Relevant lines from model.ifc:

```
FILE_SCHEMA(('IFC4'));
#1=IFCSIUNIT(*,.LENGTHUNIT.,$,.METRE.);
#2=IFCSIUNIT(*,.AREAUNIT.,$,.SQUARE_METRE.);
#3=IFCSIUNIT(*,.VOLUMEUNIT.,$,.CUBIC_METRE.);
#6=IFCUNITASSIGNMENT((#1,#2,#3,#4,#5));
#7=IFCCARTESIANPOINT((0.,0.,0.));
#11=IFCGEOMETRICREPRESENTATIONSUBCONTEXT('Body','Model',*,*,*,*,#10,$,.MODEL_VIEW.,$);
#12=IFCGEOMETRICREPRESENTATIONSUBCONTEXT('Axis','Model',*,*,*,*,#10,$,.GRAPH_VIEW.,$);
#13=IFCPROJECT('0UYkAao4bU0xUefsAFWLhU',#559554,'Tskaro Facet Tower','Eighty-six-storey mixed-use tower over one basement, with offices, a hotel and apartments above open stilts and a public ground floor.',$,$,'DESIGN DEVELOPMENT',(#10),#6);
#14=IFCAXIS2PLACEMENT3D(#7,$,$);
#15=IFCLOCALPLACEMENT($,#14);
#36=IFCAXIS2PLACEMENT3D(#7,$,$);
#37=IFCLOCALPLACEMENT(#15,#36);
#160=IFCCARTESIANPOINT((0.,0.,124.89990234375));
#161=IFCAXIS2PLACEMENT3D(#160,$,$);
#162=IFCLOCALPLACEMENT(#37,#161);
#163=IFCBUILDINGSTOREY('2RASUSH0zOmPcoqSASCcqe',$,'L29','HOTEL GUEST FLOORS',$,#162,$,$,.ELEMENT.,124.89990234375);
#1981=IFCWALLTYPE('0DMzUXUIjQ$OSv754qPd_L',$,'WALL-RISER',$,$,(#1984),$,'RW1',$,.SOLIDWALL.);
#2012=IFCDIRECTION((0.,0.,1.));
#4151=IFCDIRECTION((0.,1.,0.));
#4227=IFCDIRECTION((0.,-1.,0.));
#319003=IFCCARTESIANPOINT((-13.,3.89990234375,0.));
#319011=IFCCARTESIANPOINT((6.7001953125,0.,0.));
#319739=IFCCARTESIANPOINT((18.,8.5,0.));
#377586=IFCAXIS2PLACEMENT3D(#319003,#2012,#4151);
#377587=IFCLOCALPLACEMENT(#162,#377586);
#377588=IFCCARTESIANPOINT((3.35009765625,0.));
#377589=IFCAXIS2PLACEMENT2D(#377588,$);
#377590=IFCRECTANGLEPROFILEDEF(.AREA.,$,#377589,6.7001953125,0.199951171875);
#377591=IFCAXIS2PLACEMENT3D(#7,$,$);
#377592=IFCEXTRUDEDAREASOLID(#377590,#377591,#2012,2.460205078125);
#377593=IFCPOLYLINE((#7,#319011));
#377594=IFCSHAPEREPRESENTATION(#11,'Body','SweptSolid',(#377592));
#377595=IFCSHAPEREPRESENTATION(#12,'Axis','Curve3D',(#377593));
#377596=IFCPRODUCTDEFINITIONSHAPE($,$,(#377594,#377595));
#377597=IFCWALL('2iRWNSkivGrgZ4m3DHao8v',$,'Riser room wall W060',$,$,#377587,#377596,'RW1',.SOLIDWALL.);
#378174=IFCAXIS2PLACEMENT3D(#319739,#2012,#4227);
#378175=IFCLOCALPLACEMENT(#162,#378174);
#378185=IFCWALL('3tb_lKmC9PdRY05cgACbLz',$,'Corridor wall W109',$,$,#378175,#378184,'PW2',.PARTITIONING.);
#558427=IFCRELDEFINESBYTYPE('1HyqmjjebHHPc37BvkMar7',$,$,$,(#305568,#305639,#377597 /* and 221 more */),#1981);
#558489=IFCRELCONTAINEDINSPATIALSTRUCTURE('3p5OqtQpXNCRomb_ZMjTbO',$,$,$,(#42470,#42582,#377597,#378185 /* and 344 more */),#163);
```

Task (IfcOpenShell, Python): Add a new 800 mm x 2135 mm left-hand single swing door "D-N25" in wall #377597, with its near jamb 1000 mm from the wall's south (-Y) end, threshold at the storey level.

```python
import numpy as np
import ifcopenshell
import ifcopenshell.api.feature
import ifcopenshell.api.geometry
import ifcopenshell.api.root
import ifcopenshell.api.spatial
import ifcopenshell.geom
import ifcopenshell.util.element
import ifcopenshell.util.placement
import ifcopenshell.util.representation
import ifcopenshell.util.shape
import ifcopenshell.util.unit

model = ifcopenshell.open("model.ifc")
unit_scale = ifcopenshell.util.unit.calculate_unit_scale(model)
settings = ifcopenshell.geom.settings()


def volume(element):
    """Net volume in cubic metres, openings subtracted."""
    shape = ifcopenshell.geom.create_shape(settings, element)
    return ifcopenshell.util.shape.get_volume(shape.geometry)


wall = model.by_guid("2iRWNSkivGrgZ4m3DHao8v")
storey = ifcopenshell.util.element.get_container(wall, ifc_class="IfcBuildingStorey")
context = ifcopenshell.util.representation.get_context(model, "Model", "Body", "MODEL_VIEW")
before = volume(wall)

width, height, from_end, sill = 0.8, 2.135, 1, 0.0  # metres

# The wall runs along its own X axis, and the end named is its -X end.
wall_shape = ifcopenshell.geom.create_shape(settings, wall)
x, y, z = ifcopenshell.util.shape.get_vertices(wall_shape.geometry).T
start = x.min() + from_end
face, thickness = float(y.min()), float(y.max() - y.min())
wall_matrix = ifcopenshell.util.placement.get_local_placement(wall.ObjectPlacement)
level = ifcopenshell.util.placement.get_local_placement(storey.ObjectPlacement)[2, 3]


def in_wall(x, y):
    """Placement at x, y metres in the wall's axes, at sill height."""
    matrix = wall_matrix.copy()
    matrix[:, 3] = wall_matrix @ np.array([x / unit_scale, y / unit_scale, 0.0, 1.0])
    matrix[2, 3] = level + sill / unit_scale
    return matrix


# Opening: a box that overshoots both wall faces by 50 mm.
opening = ifcopenshell.api.root.create_entity(model, ifc_class="IfcOpeningElement", predefined_type="OPENING")
box = ifcopenshell.api.geometry.add_wall_representation(
    model, context=context, length=width, height=height, thickness=thickness + 0.1
)
ifcopenshell.api.geometry.assign_representation(model, product=opening, representation=box)
ifcopenshell.api.geometry.edit_object_placement(model, product=opening, matrix=in_wall(start, face - 0.05), is_si=False)
ifcopenshell.api.feature.add_feature(model, feature=opening, element=wall)

door = ifcopenshell.api.root.create_entity(model, ifc_class="IfcDoor", name="D-N25", predefined_type="DOOR")
door.OverallWidth, door.OverallHeight = width / unit_scale, height / unit_scale
door.OperationType = "SINGLE_SWING_LEFT"
body = ifcopenshell.api.geometry.add_door_representation(
    model,
    context=context,
    overall_width=door.OverallWidth,
    overall_height=door.OverallHeight,
    operation_type="SINGLE_SWING_LEFT",
    lining_properties={"LiningDepth": thickness / unit_scale, "ThresholdDepth": thickness / unit_scale},
)
ifcopenshell.api.geometry.assign_representation(model, product=door, representation=body)
ifcopenshell.api.spatial.assign_container(model, products=[door], relating_structure=storey)
ifcopenshell.api.feature.add_filling(model, opening=opening, element=door)

# The lining spans the wall, so the door starts at the wall face.
ifcopenshell.api.geometry.edit_object_placement(model, product=door, matrix=in_wall(start, face), is_si=False)

after = volume(wall)

print(f"wall volume {before:.3f} -> {after:.3f} m3")

model.write("model_updated.ifc")
```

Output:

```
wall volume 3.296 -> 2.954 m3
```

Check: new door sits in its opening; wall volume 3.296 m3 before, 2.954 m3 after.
